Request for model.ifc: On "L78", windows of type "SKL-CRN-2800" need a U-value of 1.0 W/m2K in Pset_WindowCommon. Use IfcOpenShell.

First a look at what the model holds.

```python
import ifcopenshell
import ifcopenshell.util.element

model = ifcopenshell.open("model.ifc")
print(model.schema)
storey = next(s for s in model.by_type("IfcBuildingStorey") if s.Name == "L78")
windows = [e for e in ifcopenshell.util.element.get_decomposition(storey) if e.is_a("IfcWindow")]
seen = {}
for e in windows:
    element_type = ifcopenshell.util.element.get_type(e)
    key = (element_type.Name if element_type != e and element_type else None, ifcopenshell.util.element.get_pset(e, "Pset_WindowCommon", "ThermalTransmittance"))
    seen[key] = seen.get(key, 0) + 1
for (name, value), count in sorted(seen.items(), key=str):
    print(count, "x", name, "|", value)
```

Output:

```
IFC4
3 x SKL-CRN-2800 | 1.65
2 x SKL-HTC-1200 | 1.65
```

```python
import ifcopenshell
import ifcopenshell.api.pset
import ifcopenshell.util.element

model = ifcopenshell.open("model.ifc")

storey = next(s for s in model.by_type("IfcBuildingStorey") if s.Name == "L78")
windows = [e for e in ifcopenshell.util.element.get_decomposition(storey) if e.is_a("IfcWindow")]

count = 0
for e in windows:
    element_type = ifcopenshell.util.element.get_type(e)
    if element_type in (None, e) or element_type.Name != "SKL-CRN-2800":
        continue
    # add_pset returns the element's existing set when there is one.
    pset = ifcopenshell.api.pset.add_pset(model, product=e, name="Pset_WindowCommon")
    ifcopenshell.api.pset.edit_pset(model, pset=pset, properties={"ThermalTransmittance": 1.0})
    count += 1

print(count, "windows updated")

model.write("model_v2.ifc")
```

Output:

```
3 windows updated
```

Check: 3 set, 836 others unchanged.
